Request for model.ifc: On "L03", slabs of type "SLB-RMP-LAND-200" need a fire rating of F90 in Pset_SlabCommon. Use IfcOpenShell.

First a look at what the model holds.

```python
import ifcopenshell
import ifcopenshell.util.element

model = ifcopenshell.open("model.ifc")
print(model.schema)
storey = next(s for s in model.by_type("IfcBuildingStorey") if s.Name == "L03")
slabs = [e for e in ifcopenshell.util.element.get_decomposition(storey) if e.is_a("IfcSlab")]
seen = {}
for e in slabs:
    element_type = ifcopenshell.util.element.get_type(e)
    key = (element_type.Name if element_type != e and element_type else None, ifcopenshell.util.element.get_pset(e, "Pset_SlabCommon", "FireRating"))
    seen[key] = seen.get(key, 0) + 1
for (name, value), count in sorted(seen.items(), key=str):
    print(count, "x", name, "|", value)
```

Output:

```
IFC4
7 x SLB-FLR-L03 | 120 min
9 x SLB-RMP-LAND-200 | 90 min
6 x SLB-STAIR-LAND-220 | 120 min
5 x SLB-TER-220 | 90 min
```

```python
import ifcopenshell
import ifcopenshell.api.pset
import ifcopenshell.util.element

model = ifcopenshell.open("model.ifc")

storey = next(s for s in model.by_type("IfcBuildingStorey") if s.Name == "L03")
slabs = [e for e in ifcopenshell.util.element.get_decomposition(storey) if e.is_a("IfcSlab")]

count = 0
for e in slabs:
    element_type = ifcopenshell.util.element.get_type(e)
    if element_type in (None, e) or element_type.Name != "SLB-RMP-LAND-200":
        continue
    # add_pset returns the element's existing set when there is one.
    pset = ifcopenshell.api.pset.add_pset(model, product=e, name="Pset_SlabCommon")
    ifcopenshell.api.pset.edit_pset(model, pset=pset, properties={"FireRating": "F90"})
    count += 1

print(count, "slabs updated")

model.write("model_rev.ifc")
```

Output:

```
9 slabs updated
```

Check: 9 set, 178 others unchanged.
